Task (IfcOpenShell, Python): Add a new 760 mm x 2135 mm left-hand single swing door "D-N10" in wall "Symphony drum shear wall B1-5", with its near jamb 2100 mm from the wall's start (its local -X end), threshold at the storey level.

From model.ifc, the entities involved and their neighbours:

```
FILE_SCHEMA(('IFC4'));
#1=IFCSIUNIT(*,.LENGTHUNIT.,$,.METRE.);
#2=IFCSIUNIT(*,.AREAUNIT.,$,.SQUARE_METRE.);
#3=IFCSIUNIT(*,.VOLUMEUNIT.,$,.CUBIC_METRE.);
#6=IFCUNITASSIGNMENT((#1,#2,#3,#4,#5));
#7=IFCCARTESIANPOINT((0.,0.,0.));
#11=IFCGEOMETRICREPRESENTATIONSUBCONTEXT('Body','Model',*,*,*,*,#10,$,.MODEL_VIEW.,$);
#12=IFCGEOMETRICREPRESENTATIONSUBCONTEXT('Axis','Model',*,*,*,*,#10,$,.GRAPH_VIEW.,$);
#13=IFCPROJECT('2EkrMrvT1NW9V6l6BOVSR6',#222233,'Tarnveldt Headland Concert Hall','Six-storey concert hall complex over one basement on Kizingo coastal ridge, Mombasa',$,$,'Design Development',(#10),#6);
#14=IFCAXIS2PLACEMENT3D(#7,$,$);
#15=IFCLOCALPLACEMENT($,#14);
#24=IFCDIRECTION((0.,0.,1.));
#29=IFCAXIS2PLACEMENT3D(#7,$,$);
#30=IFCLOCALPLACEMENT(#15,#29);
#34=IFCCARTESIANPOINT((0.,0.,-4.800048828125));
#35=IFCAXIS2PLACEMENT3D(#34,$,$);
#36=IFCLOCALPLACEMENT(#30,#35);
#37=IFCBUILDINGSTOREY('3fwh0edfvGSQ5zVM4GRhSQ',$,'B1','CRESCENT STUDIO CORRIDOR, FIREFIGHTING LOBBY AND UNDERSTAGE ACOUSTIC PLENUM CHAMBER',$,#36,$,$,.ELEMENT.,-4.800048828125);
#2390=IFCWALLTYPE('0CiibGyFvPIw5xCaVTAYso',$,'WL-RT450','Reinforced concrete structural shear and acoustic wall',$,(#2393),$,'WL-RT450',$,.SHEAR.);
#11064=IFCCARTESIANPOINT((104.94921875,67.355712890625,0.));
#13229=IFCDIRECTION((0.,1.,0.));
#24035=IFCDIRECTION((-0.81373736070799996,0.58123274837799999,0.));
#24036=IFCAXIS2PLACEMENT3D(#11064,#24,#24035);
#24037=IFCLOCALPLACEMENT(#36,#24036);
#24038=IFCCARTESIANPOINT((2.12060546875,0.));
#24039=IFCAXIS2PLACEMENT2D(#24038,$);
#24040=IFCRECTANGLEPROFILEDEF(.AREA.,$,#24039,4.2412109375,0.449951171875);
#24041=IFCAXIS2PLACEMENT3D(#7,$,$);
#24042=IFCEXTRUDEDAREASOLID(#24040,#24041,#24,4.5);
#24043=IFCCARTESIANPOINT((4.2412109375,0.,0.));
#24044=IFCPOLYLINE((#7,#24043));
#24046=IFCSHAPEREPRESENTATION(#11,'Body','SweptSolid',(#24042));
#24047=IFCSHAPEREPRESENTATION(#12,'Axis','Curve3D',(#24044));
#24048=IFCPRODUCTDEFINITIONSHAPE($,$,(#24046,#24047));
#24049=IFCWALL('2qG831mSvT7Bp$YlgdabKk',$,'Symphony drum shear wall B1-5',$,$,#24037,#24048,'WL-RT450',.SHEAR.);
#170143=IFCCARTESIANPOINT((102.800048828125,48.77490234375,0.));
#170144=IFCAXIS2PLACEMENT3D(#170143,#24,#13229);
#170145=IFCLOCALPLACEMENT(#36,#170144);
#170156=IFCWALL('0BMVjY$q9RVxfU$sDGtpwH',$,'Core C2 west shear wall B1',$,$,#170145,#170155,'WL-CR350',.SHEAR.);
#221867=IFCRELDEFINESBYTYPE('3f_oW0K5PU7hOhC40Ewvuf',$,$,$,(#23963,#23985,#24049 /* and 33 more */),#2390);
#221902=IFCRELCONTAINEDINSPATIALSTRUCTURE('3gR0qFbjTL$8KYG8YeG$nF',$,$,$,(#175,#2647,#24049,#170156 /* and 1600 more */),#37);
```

```python
import numpy as np
import ifcopenshell
import ifcopenshell.api.feature
import ifcopenshell.api.geometry
import ifcopenshell.api.root
import ifcopenshell.api.spatial
import ifcopenshell.geom
import ifcopenshell.util.element
import ifcopenshell.util.placement
import ifcopenshell.util.representation
import ifcopenshell.util.shape
import ifcopenshell.util.unit

model = ifcopenshell.open("model.ifc")
unit_scale = ifcopenshell.util.unit.calculate_unit_scale(model)
settings = ifcopenshell.geom.settings()


def volume(element):
    """Net volume in cubic metres, openings subtracted."""
    shape = ifcopenshell.geom.create_shape(settings, element)
    return ifcopenshell.util.shape.get_volume(shape.geometry)


wall = model.by_id(24049)
storey = ifcopenshell.util.element.get_container(wall, ifc_class="IfcBuildingStorey")
context = ifcopenshell.util.representation.get_context(model, "Model", "Body", "MODEL_VIEW")
before = volume(wall)

width, height, from_end, sill = 0.76, 2.135, 2.1, 0.0  # metres

# The wall runs along its own X axis, and the end named is its -X end.
wall_shape = ifcopenshell.geom.create_shape(settings, wall)
x, y, z = ifcopenshell.util.shape.get_vertices(wall_shape.geometry).T
start = x.min() + from_end
face, thickness = float(y.min()), float(y.max() - y.min())
wall_matrix = ifcopenshell.util.placement.get_local_placement(wall.ObjectPlacement)
level = ifcopenshell.util.placement.get_local_placement(storey.ObjectPlacement)[2, 3]


def in_wall(x, y):
    """Placement at x, y metres in the wall's axes, at sill height."""
    matrix = wall_matrix.copy()
    matrix[:, 3] = wall_matrix @ np.array([x / unit_scale, y / unit_scale, 0.0, 1.0])
    matrix[2, 3] = level + sill / unit_scale
    return matrix


# Opening: a box that overshoots both wall faces by 50 mm.
opening = ifcopenshell.api.root.create_entity(model, ifc_class="IfcOpeningElement", predefined_type="OPENING")
box = ifcopenshell.api.geometry.add_wall_representation(
    model, context=context, length=width, height=height, thickness=thickness + 0.1
)
ifcopenshell.api.geometry.assign_representation(model, product=opening, representation=box)
ifcopenshell.api.geometry.edit_object_placement(model, product=opening, matrix=in_wall(start, face - 0.05), is_si=False)
ifcopenshell.api.feature.add_feature(model, feature=opening, element=wall)

door = ifcopenshell.api.root.create_entity(model, ifc_class="IfcDoor", name="D-N10", predefined_type="DOOR")
door.OverallWidth, door.OverallHeight = width / unit_scale, height / unit_scale
door.OperationType = "SINGLE_SWING_LEFT"
body = ifcopenshell.api.geometry.add_door_representation(
    model,
    context=context,
    overall_width=door.OverallWidth,
    overall_height=door.OverallHeight,
    operation_type="SINGLE_SWING_LEFT",
    lining_properties={"LiningDepth": thickness / unit_scale, "ThresholdDepth": thickness / unit_scale},
)
ifcopenshell.api.geometry.assign_representation(model, product=door, representation=body)
ifcopenshell.api.spatial.assign_container(model, products=[door], relating_structure=storey)
ifcopenshell.api.feature.add_filling(model, opening=opening, element=door)

# The lining spans the wall, so the door starts at the wall face.
ifcopenshell.api.geometry.edit_object_placement(model, product=door, matrix=in_wall(start, face), is_si=False)

after = volume(wall)

print(f"wall volume {before:.3f} -> {after:.3f} m3")

model.write("model_edited.ifc")
```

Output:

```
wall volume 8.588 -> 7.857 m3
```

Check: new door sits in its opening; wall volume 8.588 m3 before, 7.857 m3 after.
